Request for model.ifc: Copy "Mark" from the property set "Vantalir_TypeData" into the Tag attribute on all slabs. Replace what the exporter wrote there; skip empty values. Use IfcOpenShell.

First a look at what the model holds.

```python
import ifcopenshell
import ifcopenshell.util.element

model = ifcopenshell.open("model.ifc")
print(model.schema)
slabs = model.by_type("IfcSlab")
print(len(slabs), "slabs")
for e in slabs[:8]:
    source = ifcopenshell.util.element.get_pset(e, "Vantalir_TypeData", "Mark")
    target = e.Tag
    print(e.id(), repr(source), repr(target), sep=" | ")
```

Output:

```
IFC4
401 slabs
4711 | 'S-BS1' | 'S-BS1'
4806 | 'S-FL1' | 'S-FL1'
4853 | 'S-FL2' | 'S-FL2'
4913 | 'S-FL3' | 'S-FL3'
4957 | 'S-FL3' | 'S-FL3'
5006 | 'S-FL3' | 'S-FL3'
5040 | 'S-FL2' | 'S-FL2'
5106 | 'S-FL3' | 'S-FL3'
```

```python
import ifcopenshell
import ifcopenshell.util.element

model = ifcopenshell.open("model.ifc")

count = 0
for e in model.by_type("IfcSlab"):
    value = ifcopenshell.util.element.get_pset(e, "Vantalir_TypeData", "Mark")
    current = e.Tag
    if not value or not value.strip() or current == value:
        continue
    e.Tag = value
    count += 1

print(count, "slabs updated")

model.write("model-out.ifc")
```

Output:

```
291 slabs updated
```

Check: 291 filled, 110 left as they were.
